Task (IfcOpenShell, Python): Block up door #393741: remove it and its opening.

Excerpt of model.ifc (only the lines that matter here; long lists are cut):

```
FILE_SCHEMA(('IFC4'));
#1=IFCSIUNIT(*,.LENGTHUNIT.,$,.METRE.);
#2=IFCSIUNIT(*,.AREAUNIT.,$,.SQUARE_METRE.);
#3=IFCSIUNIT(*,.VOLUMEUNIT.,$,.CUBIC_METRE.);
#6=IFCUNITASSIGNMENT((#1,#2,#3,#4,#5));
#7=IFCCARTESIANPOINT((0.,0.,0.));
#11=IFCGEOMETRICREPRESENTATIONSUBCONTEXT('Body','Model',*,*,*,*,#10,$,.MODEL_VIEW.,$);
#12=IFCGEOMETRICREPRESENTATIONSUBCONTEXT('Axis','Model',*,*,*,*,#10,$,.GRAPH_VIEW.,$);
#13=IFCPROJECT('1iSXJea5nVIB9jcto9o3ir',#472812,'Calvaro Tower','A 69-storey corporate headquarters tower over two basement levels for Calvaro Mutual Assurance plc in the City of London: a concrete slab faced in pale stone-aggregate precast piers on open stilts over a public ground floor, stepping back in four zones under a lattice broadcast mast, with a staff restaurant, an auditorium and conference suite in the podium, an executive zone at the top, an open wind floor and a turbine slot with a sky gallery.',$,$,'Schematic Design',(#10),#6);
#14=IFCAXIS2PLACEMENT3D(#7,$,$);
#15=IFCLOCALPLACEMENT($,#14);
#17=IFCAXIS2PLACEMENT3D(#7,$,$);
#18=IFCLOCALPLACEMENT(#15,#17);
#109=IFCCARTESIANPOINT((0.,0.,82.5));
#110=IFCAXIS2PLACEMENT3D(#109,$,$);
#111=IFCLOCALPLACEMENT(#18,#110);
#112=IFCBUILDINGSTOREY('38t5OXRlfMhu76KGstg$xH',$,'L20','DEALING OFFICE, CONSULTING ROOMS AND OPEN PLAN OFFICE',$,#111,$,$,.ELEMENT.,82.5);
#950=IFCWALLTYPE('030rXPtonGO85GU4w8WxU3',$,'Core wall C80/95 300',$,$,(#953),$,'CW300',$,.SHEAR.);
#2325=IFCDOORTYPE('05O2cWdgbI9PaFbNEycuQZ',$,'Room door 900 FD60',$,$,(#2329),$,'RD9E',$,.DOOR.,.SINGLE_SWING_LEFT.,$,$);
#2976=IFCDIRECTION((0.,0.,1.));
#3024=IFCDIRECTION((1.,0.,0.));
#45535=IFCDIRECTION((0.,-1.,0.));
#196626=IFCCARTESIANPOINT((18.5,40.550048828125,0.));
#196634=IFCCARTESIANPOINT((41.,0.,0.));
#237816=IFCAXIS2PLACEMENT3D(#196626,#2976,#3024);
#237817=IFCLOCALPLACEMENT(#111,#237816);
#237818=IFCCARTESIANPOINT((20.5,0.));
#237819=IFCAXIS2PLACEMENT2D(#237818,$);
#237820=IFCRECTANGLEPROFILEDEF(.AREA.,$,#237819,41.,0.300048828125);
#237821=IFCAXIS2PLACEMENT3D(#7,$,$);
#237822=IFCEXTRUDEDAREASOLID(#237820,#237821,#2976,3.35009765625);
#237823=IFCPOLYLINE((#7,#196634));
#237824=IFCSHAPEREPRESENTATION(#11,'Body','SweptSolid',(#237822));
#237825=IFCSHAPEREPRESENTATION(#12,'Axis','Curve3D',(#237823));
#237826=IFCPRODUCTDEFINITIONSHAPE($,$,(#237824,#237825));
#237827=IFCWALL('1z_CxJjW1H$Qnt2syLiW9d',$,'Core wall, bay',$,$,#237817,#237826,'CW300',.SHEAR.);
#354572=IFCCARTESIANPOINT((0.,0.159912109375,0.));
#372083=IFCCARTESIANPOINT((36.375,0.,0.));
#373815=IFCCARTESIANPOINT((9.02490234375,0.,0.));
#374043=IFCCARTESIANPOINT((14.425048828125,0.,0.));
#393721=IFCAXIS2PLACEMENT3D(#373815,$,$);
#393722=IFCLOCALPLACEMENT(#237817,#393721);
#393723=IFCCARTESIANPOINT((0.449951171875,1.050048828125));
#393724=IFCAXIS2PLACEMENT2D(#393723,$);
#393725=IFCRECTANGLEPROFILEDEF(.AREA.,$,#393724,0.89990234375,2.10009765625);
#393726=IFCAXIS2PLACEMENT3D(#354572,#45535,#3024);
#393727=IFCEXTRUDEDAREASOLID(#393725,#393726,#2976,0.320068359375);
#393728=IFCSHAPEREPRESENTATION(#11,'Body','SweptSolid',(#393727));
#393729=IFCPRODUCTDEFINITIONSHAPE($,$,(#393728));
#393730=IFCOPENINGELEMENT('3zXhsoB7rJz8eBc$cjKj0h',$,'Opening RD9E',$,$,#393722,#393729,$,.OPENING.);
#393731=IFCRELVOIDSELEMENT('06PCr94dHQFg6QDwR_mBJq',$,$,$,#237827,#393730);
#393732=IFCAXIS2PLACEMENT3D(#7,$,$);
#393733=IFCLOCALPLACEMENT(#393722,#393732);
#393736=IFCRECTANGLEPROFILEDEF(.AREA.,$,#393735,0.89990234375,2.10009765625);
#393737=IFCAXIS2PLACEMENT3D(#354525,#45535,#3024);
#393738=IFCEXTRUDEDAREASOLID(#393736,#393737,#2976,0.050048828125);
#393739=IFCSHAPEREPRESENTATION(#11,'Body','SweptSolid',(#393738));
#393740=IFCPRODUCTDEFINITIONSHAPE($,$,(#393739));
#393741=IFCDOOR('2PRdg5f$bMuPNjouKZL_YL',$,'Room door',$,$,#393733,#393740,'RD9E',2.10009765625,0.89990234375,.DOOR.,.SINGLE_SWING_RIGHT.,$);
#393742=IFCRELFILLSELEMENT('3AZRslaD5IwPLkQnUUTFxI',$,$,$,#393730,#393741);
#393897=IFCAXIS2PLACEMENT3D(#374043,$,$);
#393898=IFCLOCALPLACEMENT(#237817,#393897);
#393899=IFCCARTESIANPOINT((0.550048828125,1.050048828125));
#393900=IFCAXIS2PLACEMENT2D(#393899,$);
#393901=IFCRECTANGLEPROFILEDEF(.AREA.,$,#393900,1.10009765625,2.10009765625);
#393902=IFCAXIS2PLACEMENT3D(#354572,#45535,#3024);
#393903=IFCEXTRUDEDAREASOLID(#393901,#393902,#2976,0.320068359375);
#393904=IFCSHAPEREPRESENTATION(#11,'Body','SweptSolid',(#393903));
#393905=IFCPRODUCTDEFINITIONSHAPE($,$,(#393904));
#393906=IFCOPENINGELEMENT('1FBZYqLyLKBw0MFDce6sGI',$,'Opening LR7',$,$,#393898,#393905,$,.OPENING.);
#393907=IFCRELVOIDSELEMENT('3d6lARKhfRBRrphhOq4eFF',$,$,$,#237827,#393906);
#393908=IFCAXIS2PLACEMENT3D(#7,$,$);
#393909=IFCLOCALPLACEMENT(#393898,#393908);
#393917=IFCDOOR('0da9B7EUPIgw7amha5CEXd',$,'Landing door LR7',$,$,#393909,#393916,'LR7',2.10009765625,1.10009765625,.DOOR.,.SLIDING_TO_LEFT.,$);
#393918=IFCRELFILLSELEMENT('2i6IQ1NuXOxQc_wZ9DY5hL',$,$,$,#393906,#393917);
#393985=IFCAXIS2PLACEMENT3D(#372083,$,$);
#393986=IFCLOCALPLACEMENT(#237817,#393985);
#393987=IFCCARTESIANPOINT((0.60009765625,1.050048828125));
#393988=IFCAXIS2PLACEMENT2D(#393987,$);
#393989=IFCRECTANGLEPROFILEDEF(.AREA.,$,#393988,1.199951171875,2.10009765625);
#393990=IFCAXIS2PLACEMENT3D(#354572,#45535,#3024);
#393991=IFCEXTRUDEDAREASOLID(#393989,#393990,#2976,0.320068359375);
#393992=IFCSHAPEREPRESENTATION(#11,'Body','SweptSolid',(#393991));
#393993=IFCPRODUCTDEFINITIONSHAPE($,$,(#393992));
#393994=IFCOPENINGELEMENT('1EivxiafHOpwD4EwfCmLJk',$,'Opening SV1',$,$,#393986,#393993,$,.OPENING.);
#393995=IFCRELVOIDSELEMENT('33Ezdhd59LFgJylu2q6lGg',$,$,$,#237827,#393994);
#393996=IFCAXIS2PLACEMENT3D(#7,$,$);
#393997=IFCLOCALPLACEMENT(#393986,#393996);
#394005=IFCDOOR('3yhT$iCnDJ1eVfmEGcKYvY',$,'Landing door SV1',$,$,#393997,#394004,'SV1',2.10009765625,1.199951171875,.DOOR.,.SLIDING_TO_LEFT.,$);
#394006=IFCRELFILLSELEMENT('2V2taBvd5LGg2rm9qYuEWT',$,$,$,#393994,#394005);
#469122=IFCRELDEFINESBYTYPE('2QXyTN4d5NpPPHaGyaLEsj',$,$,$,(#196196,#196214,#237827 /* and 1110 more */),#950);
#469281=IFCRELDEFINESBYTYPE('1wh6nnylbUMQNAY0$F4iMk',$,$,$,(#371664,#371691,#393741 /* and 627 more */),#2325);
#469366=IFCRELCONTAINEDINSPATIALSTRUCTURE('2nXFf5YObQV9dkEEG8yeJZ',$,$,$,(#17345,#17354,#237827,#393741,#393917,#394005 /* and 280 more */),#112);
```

```python
import ifcopenshell
import ifcopenshell.api.feature
import ifcopenshell.api.root
import ifcopenshell.geom
import ifcopenshell.util.shape

model = ifcopenshell.open("model.ifc")
settings = ifcopenshell.geom.settings()


def volume(element):
    """Net volume in cubic metres, openings subtracted."""
    shape = ifcopenshell.geom.create_shape(settings, element)
    return ifcopenshell.util.shape.get_volume(shape.geometry)


door = model.by_guid("2PRdg5f$bMuPNjouKZL_YL")
opening = door.FillsVoids[0].RelatingOpeningElement
wall = opening.VoidsElements[0].RelatingBuildingElement
before = volume(wall)

ifcopenshell.api.root.remove_product(model, product=door)
ifcopenshell.api.feature.remove_feature(model, feature=opening)

after = volume(wall)

print(f"wall volume {before:.3f} -> {after:.3f} m3")

model.write("model_rev.ifc")
```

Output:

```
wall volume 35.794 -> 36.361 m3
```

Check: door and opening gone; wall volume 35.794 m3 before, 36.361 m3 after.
